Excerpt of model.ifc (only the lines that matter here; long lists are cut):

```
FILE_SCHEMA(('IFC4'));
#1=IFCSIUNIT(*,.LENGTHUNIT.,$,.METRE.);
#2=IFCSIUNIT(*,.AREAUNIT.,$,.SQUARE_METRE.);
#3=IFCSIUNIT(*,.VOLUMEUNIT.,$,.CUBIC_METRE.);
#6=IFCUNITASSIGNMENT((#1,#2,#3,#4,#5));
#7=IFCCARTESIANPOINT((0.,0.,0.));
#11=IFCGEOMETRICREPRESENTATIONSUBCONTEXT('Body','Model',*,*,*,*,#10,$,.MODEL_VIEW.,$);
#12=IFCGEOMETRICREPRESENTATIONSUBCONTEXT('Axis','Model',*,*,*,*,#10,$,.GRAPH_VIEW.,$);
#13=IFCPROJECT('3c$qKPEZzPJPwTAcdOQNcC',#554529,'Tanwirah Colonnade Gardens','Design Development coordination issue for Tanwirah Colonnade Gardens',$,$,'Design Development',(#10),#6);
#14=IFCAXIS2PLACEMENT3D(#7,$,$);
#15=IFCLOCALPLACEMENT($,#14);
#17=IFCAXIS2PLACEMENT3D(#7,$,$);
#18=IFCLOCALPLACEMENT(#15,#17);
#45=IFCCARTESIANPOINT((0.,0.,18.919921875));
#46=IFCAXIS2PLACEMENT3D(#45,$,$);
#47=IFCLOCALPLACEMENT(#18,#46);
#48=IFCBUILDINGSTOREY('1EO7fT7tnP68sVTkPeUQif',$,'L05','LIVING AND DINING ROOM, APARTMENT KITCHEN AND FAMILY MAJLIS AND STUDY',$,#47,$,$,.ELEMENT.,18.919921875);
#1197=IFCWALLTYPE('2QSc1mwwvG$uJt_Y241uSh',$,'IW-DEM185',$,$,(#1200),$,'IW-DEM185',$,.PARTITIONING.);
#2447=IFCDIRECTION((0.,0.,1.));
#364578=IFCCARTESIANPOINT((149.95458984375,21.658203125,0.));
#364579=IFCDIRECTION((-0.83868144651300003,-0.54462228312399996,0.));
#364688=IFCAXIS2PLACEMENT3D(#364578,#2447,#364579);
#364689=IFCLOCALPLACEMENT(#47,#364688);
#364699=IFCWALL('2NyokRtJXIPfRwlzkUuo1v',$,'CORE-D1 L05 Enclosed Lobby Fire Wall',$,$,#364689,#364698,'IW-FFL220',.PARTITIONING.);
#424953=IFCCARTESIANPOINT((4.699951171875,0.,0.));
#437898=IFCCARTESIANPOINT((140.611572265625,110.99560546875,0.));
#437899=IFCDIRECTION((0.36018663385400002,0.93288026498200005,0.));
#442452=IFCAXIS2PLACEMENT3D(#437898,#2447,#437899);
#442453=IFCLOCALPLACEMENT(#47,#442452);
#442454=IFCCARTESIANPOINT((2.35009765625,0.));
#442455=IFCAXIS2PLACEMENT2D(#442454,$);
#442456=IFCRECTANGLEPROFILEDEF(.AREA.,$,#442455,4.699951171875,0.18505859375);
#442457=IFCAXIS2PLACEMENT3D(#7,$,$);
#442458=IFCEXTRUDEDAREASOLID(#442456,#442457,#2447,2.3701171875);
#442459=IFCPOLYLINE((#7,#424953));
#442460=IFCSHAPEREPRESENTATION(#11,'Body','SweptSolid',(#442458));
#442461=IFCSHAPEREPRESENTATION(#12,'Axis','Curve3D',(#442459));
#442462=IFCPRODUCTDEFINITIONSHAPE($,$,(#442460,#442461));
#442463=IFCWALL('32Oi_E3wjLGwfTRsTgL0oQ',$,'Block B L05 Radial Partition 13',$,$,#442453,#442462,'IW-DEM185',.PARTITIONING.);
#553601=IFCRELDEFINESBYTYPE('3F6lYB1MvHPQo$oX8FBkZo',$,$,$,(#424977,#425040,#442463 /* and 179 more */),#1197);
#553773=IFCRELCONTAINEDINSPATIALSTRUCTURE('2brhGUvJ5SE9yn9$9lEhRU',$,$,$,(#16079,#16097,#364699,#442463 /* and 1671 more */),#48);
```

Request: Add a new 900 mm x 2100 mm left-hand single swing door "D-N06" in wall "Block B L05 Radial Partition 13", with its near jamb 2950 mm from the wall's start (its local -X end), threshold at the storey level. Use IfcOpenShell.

```python
import numpy as np
import ifcopenshell
import ifcopenshell.api.feature
import ifcopenshell.api.geometry
import ifcopenshell.api.root
import ifcopenshell.api.spatial
import ifcopenshell.geom
import ifcopenshell.util.element
import ifcopenshell.util.placement
import ifcopenshell.util.representation
import ifcopenshell.util.shape
import ifcopenshell.util.unit

model = ifcopenshell.open("model.ifc")
unit_scale = ifcopenshell.util.unit.calculate_unit_scale(model)
settings = ifcopenshell.geom.settings()


def volume(element):
    """Net volume in cubic metres, openings subtracted."""
    shape = ifcopenshell.geom.create_shape(settings, element)
    return ifcopenshell.util.shape.get_volume(shape.geometry)


wall = model.by_guid("32Oi_E3wjLGwfTRsTgL0oQ")
storey = ifcopenshell.util.element.get_container(wall, ifc_class="IfcBuildingStorey")
context = ifcopenshell.util.representation.get_context(model, "Model", "Body", "MODEL_VIEW")
before = volume(wall)

width, height, from_end, sill = 0.9, 2.1, 2.95, 0.0  # metres

# The wall runs along its own X axis, and the end named is its -X end.
wall_shape = ifcopenshell.geom.create_shape(settings, wall)
x, y, z = ifcopenshell.util.shape.get_vertices(wall_shape.geometry).T
start = x.min() + from_end
face, thickness = float(y.min()), float(y.max() - y.min())
wall_matrix = ifcopenshell.util.placement.get_local_placement(wall.ObjectPlacement)
level = ifcopenshell.util.placement.get_local_placement(storey.ObjectPlacement)[2, 3]


def in_wall(x, y):
    """Placement at x, y metres in the wall's axes, at sill height."""
    matrix = wall_matrix.copy()
    matrix[:, 3] = wall_matrix @ np.array([x / unit_scale, y / unit_scale, 0.0, 1.0])
    matrix[2, 3] = level + sill / unit_scale
    return matrix


# Opening: a box that overshoots both wall faces by 50 mm.
opening = ifcopenshell.api.root.create_entity(model, ifc_class="IfcOpeningElement", predefined_type="OPENING")
box = ifcopenshell.api.geometry.add_wall_representation(
    model, context=context, length=width, height=height, thickness=thickness + 0.1
)
ifcopenshell.api.geometry.assign_representation(model, product=opening, representation=box)
ifcopenshell.api.geometry.edit_object_placement(model, product=opening, matrix=in_wall(start, face - 0.05), is_si=False)
ifcopenshell.api.feature.add_feature(model, feature=opening, element=wall)

door = ifcopenshell.api.root.create_entity(model, ifc_class="IfcDoor", name="D-N06", predefined_type="DOOR")
door.OverallWidth, door.OverallHeight = width / unit_scale, height / unit_scale
door.OperationType = "SINGLE_SWING_LEFT"
body = ifcopenshell.api.geometry.add_door_representation(
    model,
    context=context,
    overall_width=door.OverallWidth,
    overall_height=door.OverallHeight,
    operation_type="SINGLE_SWING_LEFT",
    lining_properties={"LiningDepth": thickness / unit_scale, "ThresholdDepth": thickness / unit_scale},
)
ifcopenshell.api.geometry.assign_representation(model, product=door, representation=body)
ifcopenshell.api.spatial.assign_container(model, products=[door], relating_structure=storey)
ifcopenshell.api.feature.add_filling(model, opening=opening, element=door)

# The lining spans the wall, so the door starts at the wall face.
ifcopenshell.api.geometry.edit_object_placement(model, product=door, matrix=in_wall(start, face), is_si=False)

after = volume(wall)

print(f"wall volume {before:.3f} -> {after:.3f} m3")

model.write("model-out.ifc")
```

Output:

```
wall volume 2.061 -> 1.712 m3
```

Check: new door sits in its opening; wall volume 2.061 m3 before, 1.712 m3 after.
